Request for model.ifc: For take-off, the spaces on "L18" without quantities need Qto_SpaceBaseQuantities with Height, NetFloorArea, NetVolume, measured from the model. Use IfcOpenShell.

First a look at what the model holds.

```python
import ifcopenshell
import ifcopenshell.util.element
import ifcopenshell.util.unit

model = ifcopenshell.open("model.ifc")
print(model.schema)
for unit_type in ("LENGTHUNIT", "AREAUNIT", "VOLUMEUNIT"):
    print(unit_type, ifcopenshell.util.unit.calculate_unit_scale(model, unit_type))
storey = next(s for s in model.by_type("IfcBuildingStorey") if s.Name == "L18")
spaces = [e for e in ifcopenshell.util.element.get_decomposition(storey) if e.is_a("IfcSpace")]
for e in sorted(spaces, key=lambda e: e.id()):
    print(e.id(), e.is_a(), e.Name, list(ifcopenshell.util.element.get_psets(e, qtos_only=True)), sep=" | ")
```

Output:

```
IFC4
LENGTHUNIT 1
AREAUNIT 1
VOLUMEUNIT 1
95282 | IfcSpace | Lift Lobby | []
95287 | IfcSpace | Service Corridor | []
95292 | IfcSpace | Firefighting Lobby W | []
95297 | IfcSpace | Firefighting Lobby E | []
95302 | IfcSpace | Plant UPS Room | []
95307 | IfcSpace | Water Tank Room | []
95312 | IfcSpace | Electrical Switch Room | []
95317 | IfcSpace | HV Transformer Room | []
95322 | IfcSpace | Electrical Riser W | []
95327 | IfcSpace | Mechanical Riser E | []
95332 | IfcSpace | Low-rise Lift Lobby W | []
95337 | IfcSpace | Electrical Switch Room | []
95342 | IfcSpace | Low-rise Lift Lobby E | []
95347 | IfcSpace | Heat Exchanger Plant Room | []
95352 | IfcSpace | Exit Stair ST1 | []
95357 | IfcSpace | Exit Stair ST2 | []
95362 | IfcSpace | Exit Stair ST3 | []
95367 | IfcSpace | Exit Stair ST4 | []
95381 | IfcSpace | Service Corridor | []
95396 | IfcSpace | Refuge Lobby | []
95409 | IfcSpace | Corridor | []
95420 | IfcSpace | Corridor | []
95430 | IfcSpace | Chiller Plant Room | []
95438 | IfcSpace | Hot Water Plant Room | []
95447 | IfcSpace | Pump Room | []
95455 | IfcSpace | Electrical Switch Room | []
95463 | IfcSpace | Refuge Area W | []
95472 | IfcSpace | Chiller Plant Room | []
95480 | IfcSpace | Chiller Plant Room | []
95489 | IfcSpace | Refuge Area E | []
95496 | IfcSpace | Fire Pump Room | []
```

```python
import ifcopenshell
import ifcopenshell.api.pset
import ifcopenshell.geom
import ifcopenshell.util.element
import ifcopenshell.util.shape
import ifcopenshell.util.unit

model = ifcopenshell.open("model.ifc")
unit_scale = ifcopenshell.util.unit.calculate_unit_scale(model)
area_scale = ifcopenshell.util.unit.calculate_unit_scale(model, "AREAUNIT")
volume_scale = ifcopenshell.util.unit.calculate_unit_scale(model, "VOLUMEUNIT")
settings = ifcopenshell.geom.settings()

storey = next(s for s in model.by_type("IfcBuildingStorey") if s.Name == "L18")
spaces = [e for e in ifcopenshell.util.element.get_decomposition(storey) if e.is_a("IfcSpace")]

for e in sorted(spaces, key=lambda e: e.id()):
    if ifcopenshell.util.element.get_psets(e, qtos_only=True, should_inherit=False):
        continue
    # Geometry comes back in metres, in the element's own axes.
    shape = ifcopenshell.geom.create_shape(settings, e)
    values = {
        "Height": ifcopenshell.util.shape.get_z(shape.geometry) / unit_scale,
        "NetFloorArea": ifcopenshell.util.shape.get_footprint_area(shape.geometry) / area_scale,
        "NetVolume": ifcopenshell.util.shape.get_volume(shape.geometry) / volume_scale,
    }
    qto = ifcopenshell.api.pset.add_qto(model, product=e, name="Qto_SpaceBaseQuantities")
    ifcopenshell.api.pset.edit_qto(model, qto=qto, properties=values)
    print(e.id(), {k: round(v, 3) for k, v in values.items()})

model.write("model_updated.ifc")
```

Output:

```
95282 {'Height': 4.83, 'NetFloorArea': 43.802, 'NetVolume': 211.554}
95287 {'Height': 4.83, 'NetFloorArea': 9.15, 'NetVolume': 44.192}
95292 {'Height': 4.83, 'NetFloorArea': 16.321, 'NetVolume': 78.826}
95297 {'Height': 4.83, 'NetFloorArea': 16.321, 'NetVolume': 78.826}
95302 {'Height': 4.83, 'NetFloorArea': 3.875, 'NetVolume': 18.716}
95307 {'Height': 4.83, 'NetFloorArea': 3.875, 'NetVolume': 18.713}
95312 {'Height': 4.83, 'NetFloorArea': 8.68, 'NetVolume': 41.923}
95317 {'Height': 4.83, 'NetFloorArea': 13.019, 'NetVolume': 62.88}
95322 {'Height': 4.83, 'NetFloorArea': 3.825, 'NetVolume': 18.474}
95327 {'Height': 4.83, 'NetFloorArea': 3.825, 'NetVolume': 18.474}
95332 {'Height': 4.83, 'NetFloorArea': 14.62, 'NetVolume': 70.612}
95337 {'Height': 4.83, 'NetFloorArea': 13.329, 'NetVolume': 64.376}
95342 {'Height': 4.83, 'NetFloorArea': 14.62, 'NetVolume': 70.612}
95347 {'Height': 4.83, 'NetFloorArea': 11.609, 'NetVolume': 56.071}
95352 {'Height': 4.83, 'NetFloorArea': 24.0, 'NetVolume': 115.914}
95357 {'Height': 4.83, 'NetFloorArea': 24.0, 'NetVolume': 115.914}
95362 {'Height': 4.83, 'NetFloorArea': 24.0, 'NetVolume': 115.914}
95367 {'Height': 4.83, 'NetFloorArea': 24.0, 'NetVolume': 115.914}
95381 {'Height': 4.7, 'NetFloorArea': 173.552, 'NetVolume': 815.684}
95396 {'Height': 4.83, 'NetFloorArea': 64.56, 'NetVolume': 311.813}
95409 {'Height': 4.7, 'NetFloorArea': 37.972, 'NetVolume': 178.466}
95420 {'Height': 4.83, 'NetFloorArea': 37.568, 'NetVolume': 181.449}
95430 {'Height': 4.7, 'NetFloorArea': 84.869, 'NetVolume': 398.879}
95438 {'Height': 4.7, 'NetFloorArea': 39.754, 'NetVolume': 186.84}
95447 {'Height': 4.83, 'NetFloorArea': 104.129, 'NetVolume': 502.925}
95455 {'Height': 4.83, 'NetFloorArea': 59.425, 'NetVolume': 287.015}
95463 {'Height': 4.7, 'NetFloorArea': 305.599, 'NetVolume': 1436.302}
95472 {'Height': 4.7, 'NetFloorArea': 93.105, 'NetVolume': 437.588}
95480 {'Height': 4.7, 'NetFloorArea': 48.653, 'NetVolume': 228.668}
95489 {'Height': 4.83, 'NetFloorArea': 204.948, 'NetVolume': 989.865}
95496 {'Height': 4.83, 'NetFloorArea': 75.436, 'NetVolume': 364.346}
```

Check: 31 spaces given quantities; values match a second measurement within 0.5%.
